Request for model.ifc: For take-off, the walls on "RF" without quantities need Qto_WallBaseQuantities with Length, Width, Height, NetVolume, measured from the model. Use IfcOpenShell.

First a look at what the model holds.

```python
import ifcopenshell
import ifcopenshell.util.element
import ifcopenshell.util.unit

model = ifcopenshell.open("model.ifc")
print(model.schema)
for unit_type in ("LENGTHUNIT", "AREAUNIT", "VOLUMEUNIT"):
    print(unit_type, ifcopenshell.util.unit.calculate_unit_scale(model, unit_type))
storey = next(s for s in model.by_type("IfcBuildingStorey") if s.Name == "RF")
walls = [e for e in ifcopenshell.util.element.get_decomposition(storey) if e.is_a("IfcWall")]
for e in sorted(walls, key=lambda e: e.id()):
    print(e.id(), e.is_a(), e.Name, list(ifcopenshell.util.element.get_psets(e, qtos_only=True)), sep=" | ")
```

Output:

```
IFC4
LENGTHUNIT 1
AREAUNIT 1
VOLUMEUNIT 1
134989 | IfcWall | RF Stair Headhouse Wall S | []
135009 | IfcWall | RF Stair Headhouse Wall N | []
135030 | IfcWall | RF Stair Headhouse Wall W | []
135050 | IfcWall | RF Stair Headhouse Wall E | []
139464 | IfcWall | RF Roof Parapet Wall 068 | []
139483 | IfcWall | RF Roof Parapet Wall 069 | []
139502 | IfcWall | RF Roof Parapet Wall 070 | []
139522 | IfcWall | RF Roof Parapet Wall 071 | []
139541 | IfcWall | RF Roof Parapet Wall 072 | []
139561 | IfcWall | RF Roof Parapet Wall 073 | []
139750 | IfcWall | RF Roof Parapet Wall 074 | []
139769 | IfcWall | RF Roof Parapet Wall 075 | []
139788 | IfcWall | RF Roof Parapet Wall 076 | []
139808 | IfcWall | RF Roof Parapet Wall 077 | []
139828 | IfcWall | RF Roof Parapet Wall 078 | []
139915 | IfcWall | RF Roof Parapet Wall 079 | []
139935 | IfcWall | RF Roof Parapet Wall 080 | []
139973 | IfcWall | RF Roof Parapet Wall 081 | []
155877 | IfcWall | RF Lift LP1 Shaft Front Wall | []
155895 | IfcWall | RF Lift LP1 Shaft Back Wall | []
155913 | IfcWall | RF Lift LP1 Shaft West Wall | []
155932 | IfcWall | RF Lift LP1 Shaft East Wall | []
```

```python
import ifcopenshell
import ifcopenshell.api.pset
import ifcopenshell.geom
import ifcopenshell.util.element
import ifcopenshell.util.shape
import ifcopenshell.util.unit

model = ifcopenshell.open("model.ifc")
unit_scale = ifcopenshell.util.unit.calculate_unit_scale(model)
volume_scale = ifcopenshell.util.unit.calculate_unit_scale(model, "VOLUMEUNIT")
settings = ifcopenshell.geom.settings()

storey = next(s for s in model.by_type("IfcBuildingStorey") if s.Name == "RF")
walls = [e for e in ifcopenshell.util.element.get_decomposition(storey) if e.is_a("IfcWall")]

for e in sorted(walls, key=lambda e: e.id()):
    if ifcopenshell.util.element.get_psets(e, qtos_only=True, should_inherit=False):
        continue
    # Geometry comes back in metres, in the element's own axes.
    shape = ifcopenshell.geom.create_shape(settings, e)
    values = {
        "Length": ifcopenshell.util.shape.get_x(shape.geometry) / unit_scale,
        "Width": ifcopenshell.util.shape.get_y(shape.geometry) / unit_scale,
        "Height": ifcopenshell.util.shape.get_z(shape.geometry) / unit_scale,
        "NetVolume": ifcopenshell.util.shape.get_volume(shape.geometry) / volume_scale,
    }
    qto = ifcopenshell.api.pset.add_qto(model, product=e, name="Qto_WallBaseQuantities")
    ifcopenshell.api.pset.edit_qto(model, qto=qto, properties=values)
    print(e.id(), {k: round(v, 3) for k, v in values.items()})

model.write("model_v2.ifc")
```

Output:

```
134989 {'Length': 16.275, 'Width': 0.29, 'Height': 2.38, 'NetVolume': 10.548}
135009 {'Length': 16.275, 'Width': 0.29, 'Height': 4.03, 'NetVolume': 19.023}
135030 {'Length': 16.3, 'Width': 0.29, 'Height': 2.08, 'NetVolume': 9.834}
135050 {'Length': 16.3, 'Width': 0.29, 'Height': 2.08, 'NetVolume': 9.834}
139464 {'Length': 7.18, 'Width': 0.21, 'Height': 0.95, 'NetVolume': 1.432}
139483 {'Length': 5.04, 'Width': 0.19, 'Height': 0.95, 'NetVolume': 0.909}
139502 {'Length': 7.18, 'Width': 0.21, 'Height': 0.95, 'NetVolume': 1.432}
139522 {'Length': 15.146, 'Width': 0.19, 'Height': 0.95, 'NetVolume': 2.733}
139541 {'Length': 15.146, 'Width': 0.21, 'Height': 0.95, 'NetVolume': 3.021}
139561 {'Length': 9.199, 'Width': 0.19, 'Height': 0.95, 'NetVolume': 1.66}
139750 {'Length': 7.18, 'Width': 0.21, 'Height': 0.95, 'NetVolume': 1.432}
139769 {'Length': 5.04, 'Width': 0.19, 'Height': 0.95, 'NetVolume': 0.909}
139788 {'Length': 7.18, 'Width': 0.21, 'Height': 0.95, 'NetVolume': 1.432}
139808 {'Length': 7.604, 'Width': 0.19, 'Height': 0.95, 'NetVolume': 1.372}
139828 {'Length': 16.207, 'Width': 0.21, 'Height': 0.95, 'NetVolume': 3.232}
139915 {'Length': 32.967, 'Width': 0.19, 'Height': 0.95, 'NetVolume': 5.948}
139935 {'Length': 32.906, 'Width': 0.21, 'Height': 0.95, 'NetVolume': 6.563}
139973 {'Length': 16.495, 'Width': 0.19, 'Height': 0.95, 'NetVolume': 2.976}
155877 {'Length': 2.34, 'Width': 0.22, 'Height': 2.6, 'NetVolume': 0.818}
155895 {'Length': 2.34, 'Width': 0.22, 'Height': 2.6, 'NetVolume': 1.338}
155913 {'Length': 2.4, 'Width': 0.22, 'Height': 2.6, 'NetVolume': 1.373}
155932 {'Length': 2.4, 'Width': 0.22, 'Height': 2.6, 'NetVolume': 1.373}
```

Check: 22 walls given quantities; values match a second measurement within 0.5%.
